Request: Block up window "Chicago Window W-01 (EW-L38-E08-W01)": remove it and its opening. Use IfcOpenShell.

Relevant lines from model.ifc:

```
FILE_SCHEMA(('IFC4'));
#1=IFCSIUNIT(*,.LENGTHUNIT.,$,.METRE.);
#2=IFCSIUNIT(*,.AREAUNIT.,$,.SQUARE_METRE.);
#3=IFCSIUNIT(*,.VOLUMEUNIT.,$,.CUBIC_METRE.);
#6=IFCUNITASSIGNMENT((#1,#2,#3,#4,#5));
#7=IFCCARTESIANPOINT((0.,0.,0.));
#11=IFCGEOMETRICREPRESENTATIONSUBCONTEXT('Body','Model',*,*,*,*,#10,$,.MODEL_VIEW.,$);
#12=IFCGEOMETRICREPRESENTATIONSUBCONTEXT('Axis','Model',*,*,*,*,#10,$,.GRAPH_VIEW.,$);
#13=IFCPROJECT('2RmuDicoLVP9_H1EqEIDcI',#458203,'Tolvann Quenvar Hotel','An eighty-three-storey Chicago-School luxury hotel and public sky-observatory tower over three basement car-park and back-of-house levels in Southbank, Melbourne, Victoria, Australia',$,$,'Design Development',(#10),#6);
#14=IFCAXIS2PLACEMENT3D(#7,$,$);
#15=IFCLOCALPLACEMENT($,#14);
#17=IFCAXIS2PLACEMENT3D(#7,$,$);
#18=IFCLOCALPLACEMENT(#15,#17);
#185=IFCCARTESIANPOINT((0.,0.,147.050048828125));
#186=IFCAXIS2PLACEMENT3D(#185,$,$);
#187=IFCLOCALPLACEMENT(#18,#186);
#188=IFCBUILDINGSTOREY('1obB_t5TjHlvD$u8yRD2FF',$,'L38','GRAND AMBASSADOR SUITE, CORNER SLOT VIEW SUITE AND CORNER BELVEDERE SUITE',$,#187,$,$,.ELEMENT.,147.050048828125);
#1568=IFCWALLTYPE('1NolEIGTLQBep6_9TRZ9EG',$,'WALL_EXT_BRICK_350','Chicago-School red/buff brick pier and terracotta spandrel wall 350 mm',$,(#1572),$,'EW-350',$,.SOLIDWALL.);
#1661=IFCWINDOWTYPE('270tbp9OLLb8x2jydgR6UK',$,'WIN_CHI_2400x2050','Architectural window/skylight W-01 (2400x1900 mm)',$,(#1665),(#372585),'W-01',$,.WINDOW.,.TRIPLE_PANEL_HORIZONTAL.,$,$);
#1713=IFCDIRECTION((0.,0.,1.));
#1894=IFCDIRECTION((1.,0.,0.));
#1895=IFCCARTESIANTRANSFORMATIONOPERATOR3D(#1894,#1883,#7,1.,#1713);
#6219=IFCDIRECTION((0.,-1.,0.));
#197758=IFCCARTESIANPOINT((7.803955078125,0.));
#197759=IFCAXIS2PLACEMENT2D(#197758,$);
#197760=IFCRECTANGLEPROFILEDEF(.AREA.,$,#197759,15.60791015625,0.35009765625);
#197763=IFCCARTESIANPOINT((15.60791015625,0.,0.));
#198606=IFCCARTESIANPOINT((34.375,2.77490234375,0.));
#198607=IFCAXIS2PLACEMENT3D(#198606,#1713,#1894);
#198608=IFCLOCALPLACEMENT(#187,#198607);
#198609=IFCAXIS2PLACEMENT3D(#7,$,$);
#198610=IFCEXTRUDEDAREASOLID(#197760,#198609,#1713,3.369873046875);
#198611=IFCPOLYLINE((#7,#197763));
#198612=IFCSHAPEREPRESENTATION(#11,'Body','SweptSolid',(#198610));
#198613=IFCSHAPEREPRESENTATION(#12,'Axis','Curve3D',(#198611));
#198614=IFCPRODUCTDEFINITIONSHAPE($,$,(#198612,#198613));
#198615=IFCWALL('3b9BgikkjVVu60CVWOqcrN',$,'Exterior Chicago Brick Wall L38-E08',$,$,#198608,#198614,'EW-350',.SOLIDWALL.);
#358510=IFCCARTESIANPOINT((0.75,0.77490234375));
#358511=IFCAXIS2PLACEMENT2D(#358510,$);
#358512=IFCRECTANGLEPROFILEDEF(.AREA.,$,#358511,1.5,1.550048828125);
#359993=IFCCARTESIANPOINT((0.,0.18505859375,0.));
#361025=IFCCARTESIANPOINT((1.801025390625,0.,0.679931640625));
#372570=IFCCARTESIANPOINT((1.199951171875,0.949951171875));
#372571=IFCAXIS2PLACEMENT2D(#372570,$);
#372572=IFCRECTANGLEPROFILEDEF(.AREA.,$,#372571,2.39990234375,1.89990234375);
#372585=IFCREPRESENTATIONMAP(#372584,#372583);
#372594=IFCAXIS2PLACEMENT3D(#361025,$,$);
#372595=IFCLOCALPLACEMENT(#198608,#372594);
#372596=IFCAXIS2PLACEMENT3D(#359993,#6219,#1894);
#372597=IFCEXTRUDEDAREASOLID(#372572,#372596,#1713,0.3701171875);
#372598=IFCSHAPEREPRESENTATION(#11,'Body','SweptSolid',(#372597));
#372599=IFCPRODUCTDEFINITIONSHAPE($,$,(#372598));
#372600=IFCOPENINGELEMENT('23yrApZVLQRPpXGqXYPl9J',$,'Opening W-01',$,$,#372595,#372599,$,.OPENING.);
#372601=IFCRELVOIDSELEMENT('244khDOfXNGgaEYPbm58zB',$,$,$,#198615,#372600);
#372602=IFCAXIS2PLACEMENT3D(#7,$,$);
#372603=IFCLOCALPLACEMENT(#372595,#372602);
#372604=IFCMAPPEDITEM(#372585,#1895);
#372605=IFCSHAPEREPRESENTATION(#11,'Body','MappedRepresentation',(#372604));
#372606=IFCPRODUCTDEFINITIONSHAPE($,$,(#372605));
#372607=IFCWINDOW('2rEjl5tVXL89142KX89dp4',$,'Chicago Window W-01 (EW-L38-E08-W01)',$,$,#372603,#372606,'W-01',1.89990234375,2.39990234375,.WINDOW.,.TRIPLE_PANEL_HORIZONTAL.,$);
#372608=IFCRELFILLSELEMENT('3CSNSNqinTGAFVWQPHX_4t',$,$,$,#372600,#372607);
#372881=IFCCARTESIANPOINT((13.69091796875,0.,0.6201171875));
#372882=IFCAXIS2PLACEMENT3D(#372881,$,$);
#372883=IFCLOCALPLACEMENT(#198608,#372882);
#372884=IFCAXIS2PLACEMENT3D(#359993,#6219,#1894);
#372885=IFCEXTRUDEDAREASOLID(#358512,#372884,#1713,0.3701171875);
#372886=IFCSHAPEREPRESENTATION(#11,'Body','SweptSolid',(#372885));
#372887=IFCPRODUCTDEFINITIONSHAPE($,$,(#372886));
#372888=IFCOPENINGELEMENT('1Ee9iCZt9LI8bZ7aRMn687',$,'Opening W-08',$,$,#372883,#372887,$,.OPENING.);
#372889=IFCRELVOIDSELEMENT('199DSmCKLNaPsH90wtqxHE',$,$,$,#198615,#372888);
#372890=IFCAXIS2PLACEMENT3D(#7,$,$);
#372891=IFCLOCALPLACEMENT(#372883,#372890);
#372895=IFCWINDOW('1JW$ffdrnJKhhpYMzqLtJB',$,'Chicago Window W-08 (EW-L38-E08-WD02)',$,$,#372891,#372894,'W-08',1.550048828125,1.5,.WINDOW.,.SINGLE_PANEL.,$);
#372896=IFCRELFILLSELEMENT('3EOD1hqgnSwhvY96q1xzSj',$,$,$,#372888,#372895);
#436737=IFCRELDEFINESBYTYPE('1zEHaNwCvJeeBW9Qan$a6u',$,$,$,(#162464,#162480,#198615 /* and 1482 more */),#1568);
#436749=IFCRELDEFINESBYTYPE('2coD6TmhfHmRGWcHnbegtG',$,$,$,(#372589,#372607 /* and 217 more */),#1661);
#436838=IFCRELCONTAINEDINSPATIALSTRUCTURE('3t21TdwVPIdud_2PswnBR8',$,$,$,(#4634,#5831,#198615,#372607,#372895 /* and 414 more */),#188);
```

```python
import ifcopenshell
import ifcopenshell.api.feature
import ifcopenshell.api.root
import ifcopenshell.geom
import ifcopenshell.util.shape

model = ifcopenshell.open("model.ifc")
settings = ifcopenshell.geom.settings()


def volume(element):
    """Net volume in cubic metres, openings subtracted."""
    shape = ifcopenshell.geom.create_shape(settings, element)
    return ifcopenshell.util.shape.get_volume(shape.geometry)


window = model.by_guid("2rEjl5tVXL89142KX89dp4")
opening = window.FillsVoids[0].RelatingOpeningElement
wall = opening.VoidsElements[0].RelatingBuildingElement
before = volume(wall)

ifcopenshell.api.root.remove_product(model, product=window)
ifcopenshell.api.feature.remove_feature(model, feature=opening)

after = volume(wall)

print(f"wall volume {before:.3f} -> {after:.3f} m3")

model.write("model_rev.ifc")
```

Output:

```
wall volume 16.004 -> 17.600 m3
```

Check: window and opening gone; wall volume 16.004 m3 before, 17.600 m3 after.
